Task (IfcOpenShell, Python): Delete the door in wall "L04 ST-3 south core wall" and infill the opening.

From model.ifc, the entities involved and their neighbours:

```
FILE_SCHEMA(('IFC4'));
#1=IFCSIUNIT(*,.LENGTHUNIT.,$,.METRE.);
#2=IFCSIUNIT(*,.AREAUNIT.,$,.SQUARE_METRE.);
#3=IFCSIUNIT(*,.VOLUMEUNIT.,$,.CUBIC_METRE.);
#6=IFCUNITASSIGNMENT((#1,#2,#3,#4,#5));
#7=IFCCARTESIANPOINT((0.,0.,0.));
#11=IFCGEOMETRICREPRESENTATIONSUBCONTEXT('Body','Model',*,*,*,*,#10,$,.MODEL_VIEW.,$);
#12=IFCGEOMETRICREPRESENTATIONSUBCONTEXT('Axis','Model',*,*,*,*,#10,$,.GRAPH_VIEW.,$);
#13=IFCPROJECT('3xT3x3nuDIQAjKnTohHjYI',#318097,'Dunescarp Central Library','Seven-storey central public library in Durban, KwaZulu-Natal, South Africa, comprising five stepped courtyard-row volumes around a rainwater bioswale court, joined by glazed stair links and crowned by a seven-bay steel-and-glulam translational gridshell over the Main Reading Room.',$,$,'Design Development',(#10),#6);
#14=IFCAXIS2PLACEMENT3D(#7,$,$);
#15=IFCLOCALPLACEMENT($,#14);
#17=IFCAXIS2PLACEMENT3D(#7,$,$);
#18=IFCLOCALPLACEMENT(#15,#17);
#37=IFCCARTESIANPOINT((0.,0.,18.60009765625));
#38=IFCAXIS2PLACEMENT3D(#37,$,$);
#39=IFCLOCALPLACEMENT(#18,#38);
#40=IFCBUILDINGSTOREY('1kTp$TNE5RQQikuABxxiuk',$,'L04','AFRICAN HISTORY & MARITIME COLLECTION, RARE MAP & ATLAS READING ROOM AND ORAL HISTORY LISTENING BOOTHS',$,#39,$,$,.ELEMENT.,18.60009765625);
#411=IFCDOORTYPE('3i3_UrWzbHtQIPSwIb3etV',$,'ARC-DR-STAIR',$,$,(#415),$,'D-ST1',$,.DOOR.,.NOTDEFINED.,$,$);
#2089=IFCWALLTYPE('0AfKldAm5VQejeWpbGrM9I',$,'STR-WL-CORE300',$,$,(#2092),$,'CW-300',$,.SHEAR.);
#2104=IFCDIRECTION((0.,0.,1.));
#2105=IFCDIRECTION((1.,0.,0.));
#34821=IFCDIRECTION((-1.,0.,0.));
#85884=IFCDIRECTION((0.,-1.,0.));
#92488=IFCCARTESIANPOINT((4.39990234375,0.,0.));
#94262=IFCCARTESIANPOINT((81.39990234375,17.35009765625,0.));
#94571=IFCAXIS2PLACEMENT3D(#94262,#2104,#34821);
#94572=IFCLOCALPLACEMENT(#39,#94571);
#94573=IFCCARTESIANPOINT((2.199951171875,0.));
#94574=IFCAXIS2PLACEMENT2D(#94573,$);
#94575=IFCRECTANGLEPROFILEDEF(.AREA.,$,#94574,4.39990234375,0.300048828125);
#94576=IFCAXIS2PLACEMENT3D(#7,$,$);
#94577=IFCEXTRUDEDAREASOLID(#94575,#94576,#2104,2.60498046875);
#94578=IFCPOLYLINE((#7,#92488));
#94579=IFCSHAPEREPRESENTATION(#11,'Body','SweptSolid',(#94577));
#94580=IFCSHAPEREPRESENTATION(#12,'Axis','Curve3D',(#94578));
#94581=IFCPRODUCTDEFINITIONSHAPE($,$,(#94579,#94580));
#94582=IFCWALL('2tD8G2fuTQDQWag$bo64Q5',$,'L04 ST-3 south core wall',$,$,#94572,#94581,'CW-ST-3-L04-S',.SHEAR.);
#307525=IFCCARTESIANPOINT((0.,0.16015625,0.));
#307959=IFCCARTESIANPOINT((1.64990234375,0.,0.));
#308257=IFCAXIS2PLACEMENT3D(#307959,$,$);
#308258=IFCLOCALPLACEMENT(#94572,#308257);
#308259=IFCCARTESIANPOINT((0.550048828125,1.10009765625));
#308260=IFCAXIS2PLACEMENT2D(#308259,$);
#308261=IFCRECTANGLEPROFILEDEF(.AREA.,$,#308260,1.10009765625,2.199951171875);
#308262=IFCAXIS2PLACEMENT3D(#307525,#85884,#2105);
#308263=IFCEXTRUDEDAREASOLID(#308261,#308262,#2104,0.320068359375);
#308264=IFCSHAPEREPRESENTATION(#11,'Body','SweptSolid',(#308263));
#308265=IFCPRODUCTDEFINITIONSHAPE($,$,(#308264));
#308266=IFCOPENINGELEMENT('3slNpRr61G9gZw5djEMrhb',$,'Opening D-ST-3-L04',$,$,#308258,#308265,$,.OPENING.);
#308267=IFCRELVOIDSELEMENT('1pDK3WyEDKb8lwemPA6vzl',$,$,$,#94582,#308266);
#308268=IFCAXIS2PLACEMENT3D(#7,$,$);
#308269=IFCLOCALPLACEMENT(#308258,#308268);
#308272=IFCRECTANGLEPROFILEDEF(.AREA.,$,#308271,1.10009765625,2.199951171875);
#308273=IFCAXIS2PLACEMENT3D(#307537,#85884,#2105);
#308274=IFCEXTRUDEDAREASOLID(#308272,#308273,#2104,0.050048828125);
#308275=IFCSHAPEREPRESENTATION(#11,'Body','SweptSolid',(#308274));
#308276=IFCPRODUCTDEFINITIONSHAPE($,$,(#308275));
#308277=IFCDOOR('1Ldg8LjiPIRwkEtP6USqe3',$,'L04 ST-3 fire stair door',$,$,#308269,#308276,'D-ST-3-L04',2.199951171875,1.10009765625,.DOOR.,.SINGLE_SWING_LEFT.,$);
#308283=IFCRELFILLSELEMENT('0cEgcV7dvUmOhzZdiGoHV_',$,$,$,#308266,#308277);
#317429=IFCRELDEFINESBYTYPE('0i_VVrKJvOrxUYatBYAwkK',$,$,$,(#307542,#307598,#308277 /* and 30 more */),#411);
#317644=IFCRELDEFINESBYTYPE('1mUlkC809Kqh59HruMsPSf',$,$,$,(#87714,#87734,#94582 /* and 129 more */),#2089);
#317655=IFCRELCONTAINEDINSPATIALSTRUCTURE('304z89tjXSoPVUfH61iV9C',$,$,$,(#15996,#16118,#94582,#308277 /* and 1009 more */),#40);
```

```python
import ifcopenshell
import ifcopenshell.api.feature
import ifcopenshell.api.root
import ifcopenshell.geom
import ifcopenshell.util.shape

model = ifcopenshell.open("model.ifc")
settings = ifcopenshell.geom.settings()


def volume(element):
    """Net volume in cubic metres, openings subtracted."""
    shape = ifcopenshell.geom.create_shape(settings, element)
    return ifcopenshell.util.shape.get_volume(shape.geometry)


door = model.by_guid("1Ldg8LjiPIRwkEtP6USqe3")
opening = door.FillsVoids[0].RelatingOpeningElement
wall = opening.VoidsElements[0].RelatingBuildingElement
before = volume(wall)

ifcopenshell.api.root.remove_product(model, product=door)
ifcopenshell.api.feature.remove_feature(model, feature=opening)

after = volume(wall)

print(f"wall volume {before:.3f} -> {after:.3f} m3")

model.write("model_v2.ifc")
```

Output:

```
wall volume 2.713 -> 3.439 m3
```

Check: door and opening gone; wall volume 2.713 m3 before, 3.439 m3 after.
